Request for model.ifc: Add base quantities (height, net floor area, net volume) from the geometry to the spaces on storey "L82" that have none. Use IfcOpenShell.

First a look at what the model holds.

```python
import ifcopenshell
import ifcopenshell.util.element
import ifcopenshell.util.unit

model = ifcopenshell.open("model.ifc")
print(model.schema)
for unit_type in ("LENGTHUNIT", "AREAUNIT", "VOLUMEUNIT"):
    print(unit_type, ifcopenshell.util.unit.calculate_unit_scale(model, unit_type))
storey = next(s for s in model.by_type("IfcBuildingStorey") if s.Name == "L82")
spaces = [e for e in ifcopenshell.util.element.get_decomposition(storey) if e.is_a("IfcSpace")]
for e in sorted(spaces, key=lambda e: e.id()):
    print(e.id(), e.is_a(), e.Name, list(ifcopenshell.util.element.get_psets(e, qtos_only=True)), sep=" | ")
```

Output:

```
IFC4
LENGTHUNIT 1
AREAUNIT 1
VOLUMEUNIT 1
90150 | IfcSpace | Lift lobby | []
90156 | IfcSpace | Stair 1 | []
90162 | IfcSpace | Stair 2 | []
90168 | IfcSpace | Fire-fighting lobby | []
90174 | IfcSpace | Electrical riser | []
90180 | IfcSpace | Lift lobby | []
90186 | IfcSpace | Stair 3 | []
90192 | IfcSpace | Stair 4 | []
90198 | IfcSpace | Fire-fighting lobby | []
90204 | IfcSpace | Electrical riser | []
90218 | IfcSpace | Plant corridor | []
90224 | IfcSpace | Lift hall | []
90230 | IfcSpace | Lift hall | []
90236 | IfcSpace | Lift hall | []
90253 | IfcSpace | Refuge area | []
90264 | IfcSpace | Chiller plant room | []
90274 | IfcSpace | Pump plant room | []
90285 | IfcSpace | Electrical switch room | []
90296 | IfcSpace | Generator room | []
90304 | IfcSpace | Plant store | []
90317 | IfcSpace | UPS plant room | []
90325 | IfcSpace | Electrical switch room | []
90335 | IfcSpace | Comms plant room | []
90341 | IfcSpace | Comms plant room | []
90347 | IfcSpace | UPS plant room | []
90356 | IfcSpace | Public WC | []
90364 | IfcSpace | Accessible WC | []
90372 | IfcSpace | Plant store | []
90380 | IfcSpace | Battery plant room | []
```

```python
import ifcopenshell
import ifcopenshell.api.pset
import ifcopenshell.geom
import ifcopenshell.util.element
import ifcopenshell.util.shape
import ifcopenshell.util.unit

model = ifcopenshell.open("model.ifc")
unit_scale = ifcopenshell.util.unit.calculate_unit_scale(model)
area_scale = ifcopenshell.util.unit.calculate_unit_scale(model, "AREAUNIT")
volume_scale = ifcopenshell.util.unit.calculate_unit_scale(model, "VOLUMEUNIT")
settings = ifcopenshell.geom.settings()

storey = next(s for s in model.by_type("IfcBuildingStorey") if s.Name == "L82")
spaces = [e for e in ifcopenshell.util.element.get_decomposition(storey) if e.is_a("IfcSpace")]

for e in sorted(spaces, key=lambda e: e.id()):
    if ifcopenshell.util.element.get_psets(e, qtos_only=True, should_inherit=False):
        continue
    # Geometry comes back in metres, in the element's own axes.
    shape = ifcopenshell.geom.create_shape(settings, e)
    values = {
        "Height": ifcopenshell.util.shape.get_z(shape.geometry) / unit_scale,
        "NetFloorArea": ifcopenshell.util.shape.get_footprint_area(shape.geometry) / area_scale,
        "NetVolume": ifcopenshell.util.shape.get_volume(shape.geometry) / volume_scale,
    }
    qto = ifcopenshell.api.pset.add_qto(model, product=e, name="Qto_SpaceBaseQuantities")
    ifcopenshell.api.pset.edit_qto(model, qto=qto, properties=values)
    print(e.id(), {k: round(v, 3) for k, v in values.items()})

model.write("model_rev.ifc")
```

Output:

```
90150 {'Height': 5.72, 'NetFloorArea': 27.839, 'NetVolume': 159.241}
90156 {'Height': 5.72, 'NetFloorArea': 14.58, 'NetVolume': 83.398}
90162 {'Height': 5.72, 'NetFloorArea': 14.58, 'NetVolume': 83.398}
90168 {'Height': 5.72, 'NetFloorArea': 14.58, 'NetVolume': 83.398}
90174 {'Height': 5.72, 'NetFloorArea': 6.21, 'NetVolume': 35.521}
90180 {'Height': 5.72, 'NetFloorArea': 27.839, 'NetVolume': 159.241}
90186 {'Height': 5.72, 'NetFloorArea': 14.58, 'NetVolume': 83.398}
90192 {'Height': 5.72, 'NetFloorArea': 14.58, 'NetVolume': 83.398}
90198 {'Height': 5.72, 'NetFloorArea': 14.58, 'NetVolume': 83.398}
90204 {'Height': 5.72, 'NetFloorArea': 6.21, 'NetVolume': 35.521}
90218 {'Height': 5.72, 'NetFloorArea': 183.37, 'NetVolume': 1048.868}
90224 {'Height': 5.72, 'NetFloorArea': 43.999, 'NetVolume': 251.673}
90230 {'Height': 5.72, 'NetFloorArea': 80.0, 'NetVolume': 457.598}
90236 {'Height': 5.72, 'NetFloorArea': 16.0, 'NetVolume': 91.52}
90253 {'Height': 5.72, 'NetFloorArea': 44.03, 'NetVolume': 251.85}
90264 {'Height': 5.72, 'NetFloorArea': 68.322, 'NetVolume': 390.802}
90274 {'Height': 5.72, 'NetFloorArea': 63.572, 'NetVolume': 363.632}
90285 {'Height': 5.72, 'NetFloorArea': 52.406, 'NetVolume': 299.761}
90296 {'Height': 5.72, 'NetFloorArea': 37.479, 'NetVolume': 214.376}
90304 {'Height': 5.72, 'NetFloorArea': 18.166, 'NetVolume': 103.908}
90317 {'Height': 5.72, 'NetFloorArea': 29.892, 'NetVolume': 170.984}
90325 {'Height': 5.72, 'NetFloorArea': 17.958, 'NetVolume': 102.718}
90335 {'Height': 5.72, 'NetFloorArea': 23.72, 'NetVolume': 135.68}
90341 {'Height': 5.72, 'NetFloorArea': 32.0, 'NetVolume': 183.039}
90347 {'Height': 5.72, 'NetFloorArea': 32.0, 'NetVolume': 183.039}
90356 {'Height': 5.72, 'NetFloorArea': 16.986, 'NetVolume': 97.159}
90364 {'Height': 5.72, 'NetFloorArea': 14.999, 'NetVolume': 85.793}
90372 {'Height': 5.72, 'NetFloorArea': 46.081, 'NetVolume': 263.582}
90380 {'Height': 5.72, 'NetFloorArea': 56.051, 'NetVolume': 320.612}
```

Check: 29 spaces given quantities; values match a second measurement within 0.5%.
